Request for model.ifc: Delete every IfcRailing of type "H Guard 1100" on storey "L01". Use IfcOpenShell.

First a look at what the model holds.

```python
import ifcopenshell
import ifcopenshell.util.element

model = ifcopenshell.open("model.ifc")
print(model.schema)
storey = next(s for s in model.by_type("IfcBuildingStorey") if s.Name == "L01")
railings = [e for e in ifcopenshell.util.element.get_decomposition(storey) if e.is_a("IfcRailing")]
seen = {}
for e in railings:
    element_type = ifcopenshell.util.element.get_type(e)
    name = element_type.Name if element_type not in (None, e) else None
    seen[name] = seen.get(name, 0) + 1
for name, count in sorted(seen.items(), key=str):
    print(count, "x", name)
```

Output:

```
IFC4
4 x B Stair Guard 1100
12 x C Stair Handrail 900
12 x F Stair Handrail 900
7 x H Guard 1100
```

```python
import ifcopenshell
import ifcopenshell.api.root
import ifcopenshell.util.element

model = ifcopenshell.open("model.ifc")

storey = next(s for s in model.by_type("IfcBuildingStorey") if s.Name == "L01")
railings = [e for e in ifcopenshell.util.element.get_decomposition(storey) if e.is_a("IfcRailing")]
targets = [e for e in railings if (t := ifcopenshell.util.element.get_type(e)) not in (None, e) and t.Name == "H Guard 1100"]

for e in targets:
    ifcopenshell.api.root.remove_product(model, product=e)
print(len(targets), "removed")

model.write("model_v2.ifc")
```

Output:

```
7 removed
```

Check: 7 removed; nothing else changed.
